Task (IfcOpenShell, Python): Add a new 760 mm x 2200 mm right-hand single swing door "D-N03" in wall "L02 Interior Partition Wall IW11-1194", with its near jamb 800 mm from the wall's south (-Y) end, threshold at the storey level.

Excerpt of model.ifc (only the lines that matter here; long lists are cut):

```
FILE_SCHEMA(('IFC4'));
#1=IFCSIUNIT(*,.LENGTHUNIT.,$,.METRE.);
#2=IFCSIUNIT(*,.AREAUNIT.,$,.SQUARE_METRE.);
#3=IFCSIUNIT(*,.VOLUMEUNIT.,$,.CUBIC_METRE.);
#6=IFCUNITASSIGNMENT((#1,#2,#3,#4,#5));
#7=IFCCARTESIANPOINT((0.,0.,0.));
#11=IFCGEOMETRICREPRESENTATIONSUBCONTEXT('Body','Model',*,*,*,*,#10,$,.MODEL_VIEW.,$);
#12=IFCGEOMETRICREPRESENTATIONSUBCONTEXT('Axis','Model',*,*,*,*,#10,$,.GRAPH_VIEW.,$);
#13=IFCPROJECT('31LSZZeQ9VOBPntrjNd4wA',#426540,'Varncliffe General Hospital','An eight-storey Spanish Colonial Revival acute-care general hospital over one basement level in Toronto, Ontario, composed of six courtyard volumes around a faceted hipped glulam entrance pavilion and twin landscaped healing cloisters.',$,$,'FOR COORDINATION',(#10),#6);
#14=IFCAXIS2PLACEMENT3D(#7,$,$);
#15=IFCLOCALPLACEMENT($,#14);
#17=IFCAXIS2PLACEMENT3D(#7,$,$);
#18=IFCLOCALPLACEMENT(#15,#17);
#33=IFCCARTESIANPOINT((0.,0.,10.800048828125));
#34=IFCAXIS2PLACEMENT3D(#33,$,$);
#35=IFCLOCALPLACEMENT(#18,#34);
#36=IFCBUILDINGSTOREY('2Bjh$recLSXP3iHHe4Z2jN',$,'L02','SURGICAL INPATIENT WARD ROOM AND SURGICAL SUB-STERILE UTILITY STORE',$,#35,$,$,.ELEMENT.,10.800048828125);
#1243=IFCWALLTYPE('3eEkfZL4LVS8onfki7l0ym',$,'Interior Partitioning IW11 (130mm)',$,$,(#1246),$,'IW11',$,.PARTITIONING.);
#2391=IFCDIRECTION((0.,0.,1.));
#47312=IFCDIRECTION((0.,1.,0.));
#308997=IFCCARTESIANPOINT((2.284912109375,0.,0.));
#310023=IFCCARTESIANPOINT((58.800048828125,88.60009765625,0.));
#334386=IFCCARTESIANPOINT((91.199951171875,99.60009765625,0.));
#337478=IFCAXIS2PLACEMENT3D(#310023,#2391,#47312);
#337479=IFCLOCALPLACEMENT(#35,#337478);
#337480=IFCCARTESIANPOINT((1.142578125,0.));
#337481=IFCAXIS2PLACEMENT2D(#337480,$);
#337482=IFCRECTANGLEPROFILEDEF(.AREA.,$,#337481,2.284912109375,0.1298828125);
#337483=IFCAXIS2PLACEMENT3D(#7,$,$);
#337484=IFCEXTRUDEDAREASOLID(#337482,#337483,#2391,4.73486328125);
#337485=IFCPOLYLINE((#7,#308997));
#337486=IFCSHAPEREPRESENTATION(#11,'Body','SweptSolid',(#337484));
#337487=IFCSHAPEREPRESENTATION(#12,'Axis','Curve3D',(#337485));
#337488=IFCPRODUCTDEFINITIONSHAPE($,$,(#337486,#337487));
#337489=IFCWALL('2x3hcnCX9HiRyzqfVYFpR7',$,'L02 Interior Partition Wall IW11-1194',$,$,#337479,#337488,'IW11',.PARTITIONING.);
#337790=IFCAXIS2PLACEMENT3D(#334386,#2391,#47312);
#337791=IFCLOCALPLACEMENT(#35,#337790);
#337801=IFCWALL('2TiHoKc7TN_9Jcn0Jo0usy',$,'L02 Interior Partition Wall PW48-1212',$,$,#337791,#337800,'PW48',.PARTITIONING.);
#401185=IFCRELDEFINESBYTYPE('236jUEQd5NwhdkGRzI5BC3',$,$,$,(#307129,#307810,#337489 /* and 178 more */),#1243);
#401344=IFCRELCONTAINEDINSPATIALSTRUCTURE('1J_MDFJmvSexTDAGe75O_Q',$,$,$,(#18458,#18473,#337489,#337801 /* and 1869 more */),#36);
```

```python
import numpy as np
import ifcopenshell
import ifcopenshell.api.feature
import ifcopenshell.api.geometry
import ifcopenshell.api.root
import ifcopenshell.api.spatial
import ifcopenshell.geom
import ifcopenshell.util.element
import ifcopenshell.util.placement
import ifcopenshell.util.representation
import ifcopenshell.util.shape
import ifcopenshell.util.unit

model = ifcopenshell.open("model.ifc")
unit_scale = ifcopenshell.util.unit.calculate_unit_scale(model)
settings = ifcopenshell.geom.settings()


def volume(element):
    """Net volume in cubic metres, openings subtracted."""
    shape = ifcopenshell.geom.create_shape(settings, element)
    return ifcopenshell.util.shape.get_volume(shape.geometry)


wall = model.by_id(337489)
storey = ifcopenshell.util.element.get_container(wall, ifc_class="IfcBuildingStorey")
context = ifcopenshell.util.representation.get_context(model, "Model", "Body", "MODEL_VIEW")
before = volume(wall)

width, height, from_end, sill = 0.76, 2.2, 0.8, 0.0  # metres

# The wall runs along its own X axis, and the end named is its -X end.
wall_shape = ifcopenshell.geom.create_shape(settings, wall)
x, y, z = ifcopenshell.util.shape.get_vertices(wall_shape.geometry).T
start = x.min() + from_end
face, thickness = float(y.min()), float(y.max() - y.min())
wall_matrix = ifcopenshell.util.placement.get_local_placement(wall.ObjectPlacement)
level = ifcopenshell.util.placement.get_local_placement(storey.ObjectPlacement)[2, 3]


def in_wall(x, y):
    """Placement at x, y metres in the wall's axes, at sill height."""
    matrix = wall_matrix.copy()
    matrix[:, 3] = wall_matrix @ np.array([x / unit_scale, y / unit_scale, 0.0, 1.0])
    matrix[2, 3] = level + sill / unit_scale
    return matrix


# Opening: a box that overshoots both wall faces by 50 mm.
opening = ifcopenshell.api.root.create_entity(model, ifc_class="IfcOpeningElement", predefined_type="OPENING")
box = ifcopenshell.api.geometry.add_wall_representation(
    model, context=context, length=width, height=height, thickness=thickness + 0.1
)
ifcopenshell.api.geometry.assign_representation(model, product=opening, representation=box)
ifcopenshell.api.geometry.edit_object_placement(model, product=opening, matrix=in_wall(start, face - 0.05), is_si=False)
ifcopenshell.api.feature.add_feature(model, feature=opening, element=wall)

door = ifcopenshell.api.root.create_entity(model, ifc_class="IfcDoor", name="D-N03", predefined_type="DOOR")
door.OverallWidth, door.OverallHeight = width / unit_scale, height / unit_scale
door.OperationType = "SINGLE_SWING_RIGHT"
body = ifcopenshell.api.geometry.add_door_representation(
    model,
    context=context,
    overall_width=door.OverallWidth,
    overall_height=door.OverallHeight,
    operation_type="SINGLE_SWING_RIGHT",
    lining_properties={"LiningDepth": thickness / unit_scale, "ThresholdDepth": thickness / unit_scale},
)
ifcopenshell.api.geometry.assign_representation(model, product=door, representation=body)
ifcopenshell.api.spatial.assign_container(model, products=[door], relating_structure=storey)
ifcopenshell.api.feature.add_filling(model, opening=opening, element=door)

# The lining spans the wall, so the door starts at the wall face.
ifcopenshell.api.geometry.edit_object_placement(model, product=door, matrix=in_wall(start, face), is_si=False)

after = volume(wall)

print(f"wall volume {before:.3f} -> {after:.3f} m3")

model.write("model_updated.ifc")
```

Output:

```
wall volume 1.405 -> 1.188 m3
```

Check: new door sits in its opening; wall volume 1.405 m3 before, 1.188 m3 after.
